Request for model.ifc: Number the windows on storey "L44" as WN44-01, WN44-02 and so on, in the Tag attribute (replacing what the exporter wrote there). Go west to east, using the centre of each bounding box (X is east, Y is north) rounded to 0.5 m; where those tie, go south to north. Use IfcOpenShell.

First a look at what the model holds.

```python
import ifcopenshell
import ifcopenshell.util.element
import ifcopenshell.util.placement

model = ifcopenshell.open("model.ifc")
print(model.schema)
storey = next(s for s in model.by_type("IfcBuildingStorey") if s.Name == "L44")
windows = [e for e in ifcopenshell.util.element.get_decomposition(storey) if e.is_a("IfcWindow")]
for e in sorted(windows, key=lambda e: e.id()):
    origin = ifcopenshell.util.placement.get_local_placement(e.ObjectPlacement)[:3, 3]
    print(e.id(), e.Tag, e.Name, origin.round(2) + 0.0, sep=" | ")
```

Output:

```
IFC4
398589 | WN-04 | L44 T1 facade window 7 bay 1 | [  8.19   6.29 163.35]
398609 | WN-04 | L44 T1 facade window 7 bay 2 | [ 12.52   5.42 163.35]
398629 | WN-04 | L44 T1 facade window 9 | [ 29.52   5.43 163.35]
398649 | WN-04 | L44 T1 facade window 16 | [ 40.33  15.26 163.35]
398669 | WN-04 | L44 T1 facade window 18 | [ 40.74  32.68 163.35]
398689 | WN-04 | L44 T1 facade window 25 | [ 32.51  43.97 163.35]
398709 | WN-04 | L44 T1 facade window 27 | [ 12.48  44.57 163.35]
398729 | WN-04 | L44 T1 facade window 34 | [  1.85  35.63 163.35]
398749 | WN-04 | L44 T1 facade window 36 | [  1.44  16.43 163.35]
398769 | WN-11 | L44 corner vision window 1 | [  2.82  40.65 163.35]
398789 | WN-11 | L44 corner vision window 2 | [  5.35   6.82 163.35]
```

```python
import ifcopenshell
import ifcopenshell.geom
import ifcopenshell.util.element
import ifcopenshell.util.shape

model = ifcopenshell.open("model.ifc")
settings = ifcopenshell.geom.settings()
settings.set("use-world-coords", True)


def centre(element):
    shape = ifcopenshell.geom.create_shape(settings, element)
    return ifcopenshell.util.shape.get_bbox_centroid(shape.geometry)


storey = next(s for s in model.by_type("IfcBuildingStorey") if s.Name == "L44")
windows = [e for e in ifcopenshell.util.element.get_decomposition(storey) if e.is_a("IfcWindow")]

# Insertion points can sit at a corner or the storey origin, so sort by the geometry (in metres).
centres = {e: centre(e) for e in windows}
windows.sort(key=lambda e: (round(centres[e][0] / 0.5), centres[e][1]))

for i, e in enumerate(windows, start=1):
    number = f"WN44-{i:02d}"
    e.Tag = number
    print(e.id(), number)

model.write("model_edited.ifc")
```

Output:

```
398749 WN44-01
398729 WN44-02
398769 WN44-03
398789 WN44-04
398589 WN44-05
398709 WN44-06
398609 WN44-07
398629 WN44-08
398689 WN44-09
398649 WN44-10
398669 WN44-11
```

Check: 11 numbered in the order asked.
